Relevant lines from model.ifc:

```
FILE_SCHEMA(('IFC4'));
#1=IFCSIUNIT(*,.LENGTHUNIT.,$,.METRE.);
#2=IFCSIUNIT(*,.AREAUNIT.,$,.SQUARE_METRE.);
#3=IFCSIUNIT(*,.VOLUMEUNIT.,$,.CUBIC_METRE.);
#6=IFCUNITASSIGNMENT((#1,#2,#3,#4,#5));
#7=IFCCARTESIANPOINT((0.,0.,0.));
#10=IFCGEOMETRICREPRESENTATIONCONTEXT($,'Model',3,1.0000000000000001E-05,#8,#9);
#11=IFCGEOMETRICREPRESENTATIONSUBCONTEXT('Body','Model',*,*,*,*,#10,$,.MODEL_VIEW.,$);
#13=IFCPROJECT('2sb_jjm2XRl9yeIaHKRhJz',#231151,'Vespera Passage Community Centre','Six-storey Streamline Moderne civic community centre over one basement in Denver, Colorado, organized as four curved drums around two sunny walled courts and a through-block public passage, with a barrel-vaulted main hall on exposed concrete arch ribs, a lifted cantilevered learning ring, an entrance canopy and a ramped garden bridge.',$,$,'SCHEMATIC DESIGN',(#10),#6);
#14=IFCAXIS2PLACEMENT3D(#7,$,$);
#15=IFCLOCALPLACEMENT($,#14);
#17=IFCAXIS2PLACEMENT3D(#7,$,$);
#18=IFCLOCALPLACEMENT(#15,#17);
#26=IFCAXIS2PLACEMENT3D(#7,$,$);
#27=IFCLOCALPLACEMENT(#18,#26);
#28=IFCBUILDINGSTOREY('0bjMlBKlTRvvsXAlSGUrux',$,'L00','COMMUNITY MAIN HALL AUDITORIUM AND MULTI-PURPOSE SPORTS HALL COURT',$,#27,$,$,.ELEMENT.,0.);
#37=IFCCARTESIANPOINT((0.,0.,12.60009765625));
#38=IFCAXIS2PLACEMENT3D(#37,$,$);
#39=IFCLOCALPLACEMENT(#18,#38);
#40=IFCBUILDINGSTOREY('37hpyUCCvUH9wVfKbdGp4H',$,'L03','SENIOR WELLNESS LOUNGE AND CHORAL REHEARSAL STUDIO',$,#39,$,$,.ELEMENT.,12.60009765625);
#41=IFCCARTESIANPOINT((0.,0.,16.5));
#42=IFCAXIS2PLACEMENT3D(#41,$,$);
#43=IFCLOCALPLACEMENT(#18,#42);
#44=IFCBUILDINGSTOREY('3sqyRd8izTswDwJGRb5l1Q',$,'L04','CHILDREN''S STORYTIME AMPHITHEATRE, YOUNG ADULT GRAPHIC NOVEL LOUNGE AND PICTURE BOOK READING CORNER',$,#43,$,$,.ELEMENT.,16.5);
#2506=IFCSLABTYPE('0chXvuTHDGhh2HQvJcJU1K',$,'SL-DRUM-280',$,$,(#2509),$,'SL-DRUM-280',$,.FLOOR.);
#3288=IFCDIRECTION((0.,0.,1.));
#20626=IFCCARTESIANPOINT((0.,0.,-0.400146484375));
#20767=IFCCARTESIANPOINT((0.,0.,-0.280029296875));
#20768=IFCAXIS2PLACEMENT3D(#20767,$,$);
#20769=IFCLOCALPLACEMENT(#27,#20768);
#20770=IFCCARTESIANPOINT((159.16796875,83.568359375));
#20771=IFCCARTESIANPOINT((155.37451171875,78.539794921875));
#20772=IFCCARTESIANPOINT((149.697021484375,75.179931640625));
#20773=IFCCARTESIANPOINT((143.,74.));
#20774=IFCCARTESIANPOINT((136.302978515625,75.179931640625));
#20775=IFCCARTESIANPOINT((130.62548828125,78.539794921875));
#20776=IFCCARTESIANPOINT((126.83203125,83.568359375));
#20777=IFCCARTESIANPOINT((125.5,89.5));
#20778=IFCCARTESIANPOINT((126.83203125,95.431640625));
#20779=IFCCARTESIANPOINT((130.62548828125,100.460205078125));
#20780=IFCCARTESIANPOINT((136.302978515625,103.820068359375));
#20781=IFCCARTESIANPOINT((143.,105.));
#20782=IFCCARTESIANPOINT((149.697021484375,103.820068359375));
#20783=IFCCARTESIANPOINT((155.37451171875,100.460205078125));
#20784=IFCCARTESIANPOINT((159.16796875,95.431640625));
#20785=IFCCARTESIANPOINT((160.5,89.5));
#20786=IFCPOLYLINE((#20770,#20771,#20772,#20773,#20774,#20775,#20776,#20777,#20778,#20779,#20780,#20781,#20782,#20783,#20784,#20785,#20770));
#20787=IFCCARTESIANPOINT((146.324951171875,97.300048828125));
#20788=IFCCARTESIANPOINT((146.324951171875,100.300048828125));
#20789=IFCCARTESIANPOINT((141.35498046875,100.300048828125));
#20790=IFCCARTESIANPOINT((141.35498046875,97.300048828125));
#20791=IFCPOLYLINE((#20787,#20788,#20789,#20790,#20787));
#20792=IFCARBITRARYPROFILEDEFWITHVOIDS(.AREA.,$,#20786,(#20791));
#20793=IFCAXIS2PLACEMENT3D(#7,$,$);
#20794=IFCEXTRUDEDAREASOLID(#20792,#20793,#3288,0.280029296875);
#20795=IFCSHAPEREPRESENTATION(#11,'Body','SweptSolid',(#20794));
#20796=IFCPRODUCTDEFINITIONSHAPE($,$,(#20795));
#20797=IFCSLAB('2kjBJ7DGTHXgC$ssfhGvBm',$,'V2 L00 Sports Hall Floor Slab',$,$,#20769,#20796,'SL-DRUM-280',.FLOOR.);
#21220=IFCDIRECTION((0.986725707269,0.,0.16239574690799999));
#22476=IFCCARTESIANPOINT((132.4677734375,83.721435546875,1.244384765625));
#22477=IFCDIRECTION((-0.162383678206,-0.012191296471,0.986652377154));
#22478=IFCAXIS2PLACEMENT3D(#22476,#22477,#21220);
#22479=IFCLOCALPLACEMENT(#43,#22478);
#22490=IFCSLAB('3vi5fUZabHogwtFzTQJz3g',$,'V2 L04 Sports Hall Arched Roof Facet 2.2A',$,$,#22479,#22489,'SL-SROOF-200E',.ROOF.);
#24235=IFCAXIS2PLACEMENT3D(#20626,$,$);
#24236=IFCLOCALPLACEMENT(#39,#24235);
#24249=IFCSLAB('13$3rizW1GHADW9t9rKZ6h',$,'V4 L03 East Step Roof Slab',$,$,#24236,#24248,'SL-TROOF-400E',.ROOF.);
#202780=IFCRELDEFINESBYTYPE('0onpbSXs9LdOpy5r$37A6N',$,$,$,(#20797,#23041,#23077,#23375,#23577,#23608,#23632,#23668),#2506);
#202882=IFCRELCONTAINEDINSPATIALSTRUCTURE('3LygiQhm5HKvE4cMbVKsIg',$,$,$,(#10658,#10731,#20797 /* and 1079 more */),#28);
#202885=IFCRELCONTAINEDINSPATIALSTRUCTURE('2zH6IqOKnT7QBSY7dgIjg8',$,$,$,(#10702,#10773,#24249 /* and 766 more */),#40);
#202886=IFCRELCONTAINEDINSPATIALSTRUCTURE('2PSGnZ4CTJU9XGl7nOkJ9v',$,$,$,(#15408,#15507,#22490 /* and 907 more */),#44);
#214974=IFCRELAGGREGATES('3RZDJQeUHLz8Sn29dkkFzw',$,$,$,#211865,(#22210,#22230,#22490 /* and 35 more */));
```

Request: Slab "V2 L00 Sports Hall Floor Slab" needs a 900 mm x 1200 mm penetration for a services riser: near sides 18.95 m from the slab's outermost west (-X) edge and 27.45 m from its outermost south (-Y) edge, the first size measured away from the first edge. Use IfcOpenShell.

```python
import numpy as np
import ifcopenshell
import ifcopenshell.api.feature
import ifcopenshell.api.geometry
import ifcopenshell.api.root
import ifcopenshell.geom
import ifcopenshell.util.placement
import ifcopenshell.util.representation
import ifcopenshell.util.shape
import ifcopenshell.util.unit

model = ifcopenshell.open("model.ifc")
unit_scale = ifcopenshell.util.unit.calculate_unit_scale(model)
settings = ifcopenshell.geom.settings()


def volume(element):
    """Net volume in cubic metres, openings subtracted."""
    shape = ifcopenshell.geom.create_shape(settings, element)
    return ifcopenshell.util.shape.get_volume(shape.geometry)


slab = model.by_guid("2kjBJ7DGTHXgC$ssfhGvBm")
before = volume(slab)

# Extent in the slab's own axes, in metres. The edges named are its -X and -Y sides.
slab_shape = ifcopenshell.geom.create_shape(settings, slab)
vertices = ifcopenshell.util.shape.get_vertices(slab_shape.geometry)
x_min, y_min, bottom = vertices.min(axis=0)
top = vertices[:, 2].max()

opening = ifcopenshell.api.root.create_entity(model, ifc_class="IfcOpeningElement", name="Services riser opening", predefined_type="OPENING")
context = ifcopenshell.util.representation.get_context(model, "Model", "Body", "MODEL_VIEW")
width, depth = 0.9, 1.2
outline = [(0.0, 0.0), (width, 0.0), (width, depth), (0.0, depth), (0.0, 0.0)]
# Overshoot both faces by 50 mm so the cut is clean.
shape = ifcopenshell.api.geometry.add_slab_representation(
    model, context=context, depth=top - bottom + 0.1, polyline=outline
)
ifcopenshell.api.geometry.assign_representation(model, product=opening, representation=shape)

matrix = ifcopenshell.util.placement.get_local_placement(slab.ObjectPlacement)
matrix[:, 3] = matrix @ np.append(np.array([x_min + 18.95, y_min + 27.45, bottom - 0.05]) / unit_scale, 1.0)
ifcopenshell.api.geometry.edit_object_placement(model, product=opening, matrix=matrix, is_si=False)
ifcopenshell.api.feature.add_feature(model, feature=opening, element=slab)

after = volume(slab)

print(f"slab volume {before:.3f} -> {after:.3f} m3")

model.write("model_updated.ifc")
```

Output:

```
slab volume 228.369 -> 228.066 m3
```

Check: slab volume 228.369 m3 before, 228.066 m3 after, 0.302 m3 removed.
